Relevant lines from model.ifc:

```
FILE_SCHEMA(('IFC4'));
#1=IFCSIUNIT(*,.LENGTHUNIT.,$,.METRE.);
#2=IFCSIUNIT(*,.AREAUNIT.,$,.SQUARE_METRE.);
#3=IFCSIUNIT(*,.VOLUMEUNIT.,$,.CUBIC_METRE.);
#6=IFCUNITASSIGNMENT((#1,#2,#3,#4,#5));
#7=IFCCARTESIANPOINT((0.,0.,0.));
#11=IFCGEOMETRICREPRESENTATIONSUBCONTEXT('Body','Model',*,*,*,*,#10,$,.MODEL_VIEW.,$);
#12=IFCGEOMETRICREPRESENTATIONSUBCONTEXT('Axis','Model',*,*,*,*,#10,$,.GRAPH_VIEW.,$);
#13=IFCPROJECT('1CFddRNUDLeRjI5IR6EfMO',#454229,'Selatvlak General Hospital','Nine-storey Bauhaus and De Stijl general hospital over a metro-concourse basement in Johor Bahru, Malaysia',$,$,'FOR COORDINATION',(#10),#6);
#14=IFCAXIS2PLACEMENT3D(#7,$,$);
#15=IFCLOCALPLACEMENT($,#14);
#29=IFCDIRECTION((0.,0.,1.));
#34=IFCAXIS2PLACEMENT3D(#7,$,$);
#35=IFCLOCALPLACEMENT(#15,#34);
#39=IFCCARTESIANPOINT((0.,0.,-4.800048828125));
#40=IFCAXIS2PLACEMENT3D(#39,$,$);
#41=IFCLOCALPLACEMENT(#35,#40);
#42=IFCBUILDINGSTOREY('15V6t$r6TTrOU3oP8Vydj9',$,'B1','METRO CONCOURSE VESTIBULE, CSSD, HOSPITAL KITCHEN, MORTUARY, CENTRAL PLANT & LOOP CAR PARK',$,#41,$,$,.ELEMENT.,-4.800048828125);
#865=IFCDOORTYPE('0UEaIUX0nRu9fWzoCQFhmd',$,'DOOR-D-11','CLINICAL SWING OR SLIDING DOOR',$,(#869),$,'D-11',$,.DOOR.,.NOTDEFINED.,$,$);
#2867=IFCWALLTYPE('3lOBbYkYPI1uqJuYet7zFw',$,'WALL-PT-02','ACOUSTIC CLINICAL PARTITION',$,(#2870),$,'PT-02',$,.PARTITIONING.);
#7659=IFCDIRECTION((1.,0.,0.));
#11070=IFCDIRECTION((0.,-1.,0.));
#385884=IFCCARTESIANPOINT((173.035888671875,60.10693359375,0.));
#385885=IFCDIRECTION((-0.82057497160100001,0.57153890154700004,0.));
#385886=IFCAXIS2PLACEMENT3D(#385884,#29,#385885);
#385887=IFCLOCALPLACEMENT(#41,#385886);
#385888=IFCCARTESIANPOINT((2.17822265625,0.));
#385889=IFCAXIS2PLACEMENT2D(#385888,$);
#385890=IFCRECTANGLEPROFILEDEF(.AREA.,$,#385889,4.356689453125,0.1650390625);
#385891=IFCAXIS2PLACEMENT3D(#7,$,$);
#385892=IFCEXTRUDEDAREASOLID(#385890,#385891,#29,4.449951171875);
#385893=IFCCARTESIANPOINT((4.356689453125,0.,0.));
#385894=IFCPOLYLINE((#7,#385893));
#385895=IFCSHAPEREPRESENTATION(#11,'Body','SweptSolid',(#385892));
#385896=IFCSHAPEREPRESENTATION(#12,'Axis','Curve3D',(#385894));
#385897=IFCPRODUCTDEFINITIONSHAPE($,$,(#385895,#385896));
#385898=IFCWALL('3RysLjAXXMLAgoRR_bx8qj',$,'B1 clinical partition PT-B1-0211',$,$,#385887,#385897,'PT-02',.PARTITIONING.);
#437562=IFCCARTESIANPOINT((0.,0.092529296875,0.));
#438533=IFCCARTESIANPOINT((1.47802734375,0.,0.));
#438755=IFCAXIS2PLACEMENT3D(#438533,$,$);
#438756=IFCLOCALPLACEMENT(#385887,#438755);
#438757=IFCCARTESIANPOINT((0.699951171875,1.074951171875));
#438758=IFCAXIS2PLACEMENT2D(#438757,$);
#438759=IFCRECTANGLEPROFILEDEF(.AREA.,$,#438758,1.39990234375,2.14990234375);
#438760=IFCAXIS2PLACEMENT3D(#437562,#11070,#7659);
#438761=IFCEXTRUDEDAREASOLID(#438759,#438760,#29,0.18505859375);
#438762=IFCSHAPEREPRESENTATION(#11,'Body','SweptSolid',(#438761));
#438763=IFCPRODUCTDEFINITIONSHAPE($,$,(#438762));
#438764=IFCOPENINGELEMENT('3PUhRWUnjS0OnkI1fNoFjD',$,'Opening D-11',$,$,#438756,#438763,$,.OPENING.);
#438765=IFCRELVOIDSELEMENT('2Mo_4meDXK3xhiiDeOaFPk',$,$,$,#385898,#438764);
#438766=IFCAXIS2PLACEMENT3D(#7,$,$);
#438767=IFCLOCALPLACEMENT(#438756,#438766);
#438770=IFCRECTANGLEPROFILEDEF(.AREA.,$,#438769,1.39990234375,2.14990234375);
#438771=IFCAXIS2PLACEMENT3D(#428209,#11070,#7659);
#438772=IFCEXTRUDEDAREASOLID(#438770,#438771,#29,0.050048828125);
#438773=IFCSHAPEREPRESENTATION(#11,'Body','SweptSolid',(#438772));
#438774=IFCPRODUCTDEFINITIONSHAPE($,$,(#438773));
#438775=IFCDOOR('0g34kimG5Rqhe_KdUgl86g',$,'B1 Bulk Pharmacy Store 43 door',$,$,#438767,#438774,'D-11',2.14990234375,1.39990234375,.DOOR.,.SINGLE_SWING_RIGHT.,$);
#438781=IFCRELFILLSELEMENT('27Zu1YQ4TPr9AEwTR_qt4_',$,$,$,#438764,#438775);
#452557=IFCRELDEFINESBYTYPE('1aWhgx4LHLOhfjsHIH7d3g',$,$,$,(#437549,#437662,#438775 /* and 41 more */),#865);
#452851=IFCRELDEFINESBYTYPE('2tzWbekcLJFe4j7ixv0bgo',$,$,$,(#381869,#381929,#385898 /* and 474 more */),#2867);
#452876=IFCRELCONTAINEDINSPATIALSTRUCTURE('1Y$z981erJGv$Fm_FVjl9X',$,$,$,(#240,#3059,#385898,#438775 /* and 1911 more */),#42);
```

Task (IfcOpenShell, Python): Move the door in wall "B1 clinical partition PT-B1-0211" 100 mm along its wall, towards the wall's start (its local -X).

```python
import ifcopenshell
import ifcopenshell.api.geometry
import ifcopenshell.util.placement
import ifcopenshell.util.unit

model = ifcopenshell.open("model.ifc")
unit_scale = ifcopenshell.util.unit.calculate_unit_scale(model)

door = model.by_guid("0g34kimG5Rqhe_KdUgl86g")
opening = door.FillsVoids[0].RelatingOpeningElement
wall = opening.VoidsElements[0].RelatingBuildingElement

wall_matrix = ifcopenshell.util.placement.get_local_placement(wall.ObjectPlacement)
shift = wall_matrix[:3, 0] * -0.1 / unit_scale
before = ifcopenshell.util.placement.get_local_placement(door.ObjectPlacement)[:3, 3].copy()

# The door is placed relative to its opening, so it follows when the opening moves.
matrix = ifcopenshell.util.placement.get_local_placement(opening.ObjectPlacement)
matrix[:3, 3] += shift
ifcopenshell.api.geometry.edit_object_placement(
    model, product=opening, matrix=matrix, is_si=False, should_transform_children=True
)

after = ifcopenshell.util.placement.get_local_placement(door.ObjectPlacement)[:3, 3]
print("door moved by", (after - before).round(3) + 0.0)

model.write("model-out.ifc")
```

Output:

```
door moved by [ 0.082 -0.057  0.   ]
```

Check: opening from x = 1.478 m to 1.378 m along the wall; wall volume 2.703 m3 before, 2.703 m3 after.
